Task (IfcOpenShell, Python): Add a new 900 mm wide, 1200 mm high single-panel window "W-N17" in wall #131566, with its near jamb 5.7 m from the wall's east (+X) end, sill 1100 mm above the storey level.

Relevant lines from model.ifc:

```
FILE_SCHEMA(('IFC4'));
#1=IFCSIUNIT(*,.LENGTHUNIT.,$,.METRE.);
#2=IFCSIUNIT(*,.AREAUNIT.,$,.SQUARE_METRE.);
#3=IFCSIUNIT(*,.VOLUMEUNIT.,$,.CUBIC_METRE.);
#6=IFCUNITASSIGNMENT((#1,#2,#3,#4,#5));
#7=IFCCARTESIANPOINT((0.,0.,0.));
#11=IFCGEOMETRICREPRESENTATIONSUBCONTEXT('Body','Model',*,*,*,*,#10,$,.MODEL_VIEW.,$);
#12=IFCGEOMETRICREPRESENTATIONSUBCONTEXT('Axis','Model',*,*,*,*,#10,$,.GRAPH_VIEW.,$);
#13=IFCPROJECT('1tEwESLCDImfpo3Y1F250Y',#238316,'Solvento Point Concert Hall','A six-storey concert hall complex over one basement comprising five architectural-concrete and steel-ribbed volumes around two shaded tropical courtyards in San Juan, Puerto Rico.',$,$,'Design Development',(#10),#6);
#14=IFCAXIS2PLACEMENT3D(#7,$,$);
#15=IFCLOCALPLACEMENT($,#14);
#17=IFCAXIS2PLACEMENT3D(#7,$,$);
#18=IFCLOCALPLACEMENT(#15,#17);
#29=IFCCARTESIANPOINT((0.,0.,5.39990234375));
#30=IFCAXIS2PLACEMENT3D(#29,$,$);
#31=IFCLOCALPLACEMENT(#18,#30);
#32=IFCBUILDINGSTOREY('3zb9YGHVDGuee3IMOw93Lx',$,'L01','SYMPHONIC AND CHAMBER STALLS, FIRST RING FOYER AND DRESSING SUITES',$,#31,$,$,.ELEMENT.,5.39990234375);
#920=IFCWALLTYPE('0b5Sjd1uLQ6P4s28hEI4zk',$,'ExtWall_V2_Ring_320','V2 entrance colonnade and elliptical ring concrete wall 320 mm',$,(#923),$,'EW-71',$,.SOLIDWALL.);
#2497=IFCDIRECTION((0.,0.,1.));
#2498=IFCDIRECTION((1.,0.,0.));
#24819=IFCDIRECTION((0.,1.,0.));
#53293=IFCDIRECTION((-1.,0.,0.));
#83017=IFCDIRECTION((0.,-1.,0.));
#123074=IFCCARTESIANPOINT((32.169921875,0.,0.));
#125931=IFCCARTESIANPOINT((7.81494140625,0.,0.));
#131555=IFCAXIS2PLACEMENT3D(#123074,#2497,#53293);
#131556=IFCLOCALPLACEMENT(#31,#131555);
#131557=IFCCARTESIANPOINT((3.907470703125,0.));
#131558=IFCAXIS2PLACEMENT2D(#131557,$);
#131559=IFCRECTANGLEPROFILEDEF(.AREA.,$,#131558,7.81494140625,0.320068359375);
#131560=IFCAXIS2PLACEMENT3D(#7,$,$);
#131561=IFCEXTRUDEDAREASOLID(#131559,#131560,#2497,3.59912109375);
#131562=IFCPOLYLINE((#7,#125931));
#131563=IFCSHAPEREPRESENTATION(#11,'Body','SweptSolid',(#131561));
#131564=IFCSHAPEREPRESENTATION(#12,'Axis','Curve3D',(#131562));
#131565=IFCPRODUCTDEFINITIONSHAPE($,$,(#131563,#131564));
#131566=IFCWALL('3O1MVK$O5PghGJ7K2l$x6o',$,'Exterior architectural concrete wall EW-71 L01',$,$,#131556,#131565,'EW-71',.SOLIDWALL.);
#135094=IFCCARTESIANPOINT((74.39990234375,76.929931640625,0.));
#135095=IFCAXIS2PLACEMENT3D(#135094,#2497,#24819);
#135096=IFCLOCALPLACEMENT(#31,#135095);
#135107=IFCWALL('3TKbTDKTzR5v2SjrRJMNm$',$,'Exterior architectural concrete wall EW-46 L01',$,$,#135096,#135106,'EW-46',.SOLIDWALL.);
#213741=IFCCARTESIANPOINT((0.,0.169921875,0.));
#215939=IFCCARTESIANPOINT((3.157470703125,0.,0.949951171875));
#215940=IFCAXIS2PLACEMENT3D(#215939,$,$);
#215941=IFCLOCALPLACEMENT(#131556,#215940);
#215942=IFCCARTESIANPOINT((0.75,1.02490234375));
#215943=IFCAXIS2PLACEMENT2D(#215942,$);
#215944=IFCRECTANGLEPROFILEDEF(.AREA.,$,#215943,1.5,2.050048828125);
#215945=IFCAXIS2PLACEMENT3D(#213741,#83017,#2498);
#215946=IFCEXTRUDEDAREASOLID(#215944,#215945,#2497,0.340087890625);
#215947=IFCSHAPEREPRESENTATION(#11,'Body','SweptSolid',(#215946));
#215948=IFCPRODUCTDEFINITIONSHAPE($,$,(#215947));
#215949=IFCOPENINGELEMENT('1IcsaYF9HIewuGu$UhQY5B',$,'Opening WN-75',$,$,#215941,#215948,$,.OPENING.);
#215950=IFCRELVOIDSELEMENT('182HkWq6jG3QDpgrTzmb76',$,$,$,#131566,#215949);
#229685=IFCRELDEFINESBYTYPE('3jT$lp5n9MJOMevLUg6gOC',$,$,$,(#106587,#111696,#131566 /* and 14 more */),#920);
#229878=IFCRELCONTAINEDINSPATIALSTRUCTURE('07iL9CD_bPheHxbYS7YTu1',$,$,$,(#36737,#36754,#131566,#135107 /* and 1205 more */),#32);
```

```python
import numpy as np
import ifcopenshell
import ifcopenshell.api.feature
import ifcopenshell.api.geometry
import ifcopenshell.api.root
import ifcopenshell.api.spatial
import ifcopenshell.geom
import ifcopenshell.util.element
import ifcopenshell.util.placement
import ifcopenshell.util.representation
import ifcopenshell.util.shape
import ifcopenshell.util.unit

model = ifcopenshell.open("model.ifc")
unit_scale = ifcopenshell.util.unit.calculate_unit_scale(model)
settings = ifcopenshell.geom.settings()


def volume(element):
    """Net volume in cubic metres, openings subtracted."""
    shape = ifcopenshell.geom.create_shape(settings, element)
    return ifcopenshell.util.shape.get_volume(shape.geometry)


wall = model.by_guid("3O1MVK$O5PghGJ7K2l$x6o")
storey = ifcopenshell.util.element.get_container(wall, ifc_class="IfcBuildingStorey")
context = ifcopenshell.util.representation.get_context(model, "Model", "Body", "MODEL_VIEW")
before = volume(wall)

width, height, from_end, sill = 0.9, 1.2, 5.7, 1.1  # metres

# The wall runs along its own X axis, and the end named is its -X end.
wall_shape = ifcopenshell.geom.create_shape(settings, wall)
x, y, z = ifcopenshell.util.shape.get_vertices(wall_shape.geometry).T
start = x.min() + from_end
face, thickness = float(y.min()), float(y.max() - y.min())
wall_matrix = ifcopenshell.util.placement.get_local_placement(wall.ObjectPlacement)
level = ifcopenshell.util.placement.get_local_placement(storey.ObjectPlacement)[2, 3]


def in_wall(x, y):
    """Placement at x, y metres in the wall's axes, at sill height."""
    matrix = wall_matrix.copy()
    matrix[:, 3] = wall_matrix @ np.array([x / unit_scale, y / unit_scale, 0.0, 1.0])
    matrix[2, 3] = level + sill / unit_scale
    return matrix


# Opening: a box that overshoots both wall faces by 50 mm.
opening = ifcopenshell.api.root.create_entity(model, ifc_class="IfcOpeningElement", predefined_type="OPENING")
box = ifcopenshell.api.geometry.add_wall_representation(
    model, context=context, length=width, height=height, thickness=thickness + 0.1
)
ifcopenshell.api.geometry.assign_representation(model, product=opening, representation=box)
ifcopenshell.api.geometry.edit_object_placement(model, product=opening, matrix=in_wall(start, face - 0.05), is_si=False)
ifcopenshell.api.feature.add_feature(model, feature=opening, element=wall)

window = ifcopenshell.api.root.create_entity(model, ifc_class="IfcWindow", name="W-N17", predefined_type="WINDOW")
window.OverallWidth, window.OverallHeight = width / unit_scale, height / unit_scale
window.PartitioningType = "SINGLE_PANEL"
body = ifcopenshell.api.geometry.add_window_representation(
    model,
    context=context,
    overall_width=window.OverallWidth,
    overall_height=window.OverallHeight,
    partition_type="SINGLE_PANEL",
)
ifcopenshell.api.geometry.assign_representation(model, product=window, representation=body)
ifcopenshell.api.spatial.assign_container(model, products=[window], relating_structure=storey)
ifcopenshell.api.feature.add_filling(model, opening=opening, element=window)

# Centre the window in the wall's thickness.
ifcopenshell.api.geometry.edit_object_placement(model, product=window, matrix=in_wall(start, face), is_si=False)
window_shape = ifcopenshell.geom.create_shape(settings, window)
depth = ifcopenshell.util.shape.get_vertices(window_shape.geometry)[:, 1]
offset = face + thickness / 2 - (depth.min() + depth.max()) / 2
ifcopenshell.api.geometry.edit_object_placement(model, product=window, matrix=in_wall(start, offset), is_si=False)

after = volume(wall)

print(f"wall volume {before:.3f} -> {after:.3f} m3")

model.write("model_v2.ifc")
```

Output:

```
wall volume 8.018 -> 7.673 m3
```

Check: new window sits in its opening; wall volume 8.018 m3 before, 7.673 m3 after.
